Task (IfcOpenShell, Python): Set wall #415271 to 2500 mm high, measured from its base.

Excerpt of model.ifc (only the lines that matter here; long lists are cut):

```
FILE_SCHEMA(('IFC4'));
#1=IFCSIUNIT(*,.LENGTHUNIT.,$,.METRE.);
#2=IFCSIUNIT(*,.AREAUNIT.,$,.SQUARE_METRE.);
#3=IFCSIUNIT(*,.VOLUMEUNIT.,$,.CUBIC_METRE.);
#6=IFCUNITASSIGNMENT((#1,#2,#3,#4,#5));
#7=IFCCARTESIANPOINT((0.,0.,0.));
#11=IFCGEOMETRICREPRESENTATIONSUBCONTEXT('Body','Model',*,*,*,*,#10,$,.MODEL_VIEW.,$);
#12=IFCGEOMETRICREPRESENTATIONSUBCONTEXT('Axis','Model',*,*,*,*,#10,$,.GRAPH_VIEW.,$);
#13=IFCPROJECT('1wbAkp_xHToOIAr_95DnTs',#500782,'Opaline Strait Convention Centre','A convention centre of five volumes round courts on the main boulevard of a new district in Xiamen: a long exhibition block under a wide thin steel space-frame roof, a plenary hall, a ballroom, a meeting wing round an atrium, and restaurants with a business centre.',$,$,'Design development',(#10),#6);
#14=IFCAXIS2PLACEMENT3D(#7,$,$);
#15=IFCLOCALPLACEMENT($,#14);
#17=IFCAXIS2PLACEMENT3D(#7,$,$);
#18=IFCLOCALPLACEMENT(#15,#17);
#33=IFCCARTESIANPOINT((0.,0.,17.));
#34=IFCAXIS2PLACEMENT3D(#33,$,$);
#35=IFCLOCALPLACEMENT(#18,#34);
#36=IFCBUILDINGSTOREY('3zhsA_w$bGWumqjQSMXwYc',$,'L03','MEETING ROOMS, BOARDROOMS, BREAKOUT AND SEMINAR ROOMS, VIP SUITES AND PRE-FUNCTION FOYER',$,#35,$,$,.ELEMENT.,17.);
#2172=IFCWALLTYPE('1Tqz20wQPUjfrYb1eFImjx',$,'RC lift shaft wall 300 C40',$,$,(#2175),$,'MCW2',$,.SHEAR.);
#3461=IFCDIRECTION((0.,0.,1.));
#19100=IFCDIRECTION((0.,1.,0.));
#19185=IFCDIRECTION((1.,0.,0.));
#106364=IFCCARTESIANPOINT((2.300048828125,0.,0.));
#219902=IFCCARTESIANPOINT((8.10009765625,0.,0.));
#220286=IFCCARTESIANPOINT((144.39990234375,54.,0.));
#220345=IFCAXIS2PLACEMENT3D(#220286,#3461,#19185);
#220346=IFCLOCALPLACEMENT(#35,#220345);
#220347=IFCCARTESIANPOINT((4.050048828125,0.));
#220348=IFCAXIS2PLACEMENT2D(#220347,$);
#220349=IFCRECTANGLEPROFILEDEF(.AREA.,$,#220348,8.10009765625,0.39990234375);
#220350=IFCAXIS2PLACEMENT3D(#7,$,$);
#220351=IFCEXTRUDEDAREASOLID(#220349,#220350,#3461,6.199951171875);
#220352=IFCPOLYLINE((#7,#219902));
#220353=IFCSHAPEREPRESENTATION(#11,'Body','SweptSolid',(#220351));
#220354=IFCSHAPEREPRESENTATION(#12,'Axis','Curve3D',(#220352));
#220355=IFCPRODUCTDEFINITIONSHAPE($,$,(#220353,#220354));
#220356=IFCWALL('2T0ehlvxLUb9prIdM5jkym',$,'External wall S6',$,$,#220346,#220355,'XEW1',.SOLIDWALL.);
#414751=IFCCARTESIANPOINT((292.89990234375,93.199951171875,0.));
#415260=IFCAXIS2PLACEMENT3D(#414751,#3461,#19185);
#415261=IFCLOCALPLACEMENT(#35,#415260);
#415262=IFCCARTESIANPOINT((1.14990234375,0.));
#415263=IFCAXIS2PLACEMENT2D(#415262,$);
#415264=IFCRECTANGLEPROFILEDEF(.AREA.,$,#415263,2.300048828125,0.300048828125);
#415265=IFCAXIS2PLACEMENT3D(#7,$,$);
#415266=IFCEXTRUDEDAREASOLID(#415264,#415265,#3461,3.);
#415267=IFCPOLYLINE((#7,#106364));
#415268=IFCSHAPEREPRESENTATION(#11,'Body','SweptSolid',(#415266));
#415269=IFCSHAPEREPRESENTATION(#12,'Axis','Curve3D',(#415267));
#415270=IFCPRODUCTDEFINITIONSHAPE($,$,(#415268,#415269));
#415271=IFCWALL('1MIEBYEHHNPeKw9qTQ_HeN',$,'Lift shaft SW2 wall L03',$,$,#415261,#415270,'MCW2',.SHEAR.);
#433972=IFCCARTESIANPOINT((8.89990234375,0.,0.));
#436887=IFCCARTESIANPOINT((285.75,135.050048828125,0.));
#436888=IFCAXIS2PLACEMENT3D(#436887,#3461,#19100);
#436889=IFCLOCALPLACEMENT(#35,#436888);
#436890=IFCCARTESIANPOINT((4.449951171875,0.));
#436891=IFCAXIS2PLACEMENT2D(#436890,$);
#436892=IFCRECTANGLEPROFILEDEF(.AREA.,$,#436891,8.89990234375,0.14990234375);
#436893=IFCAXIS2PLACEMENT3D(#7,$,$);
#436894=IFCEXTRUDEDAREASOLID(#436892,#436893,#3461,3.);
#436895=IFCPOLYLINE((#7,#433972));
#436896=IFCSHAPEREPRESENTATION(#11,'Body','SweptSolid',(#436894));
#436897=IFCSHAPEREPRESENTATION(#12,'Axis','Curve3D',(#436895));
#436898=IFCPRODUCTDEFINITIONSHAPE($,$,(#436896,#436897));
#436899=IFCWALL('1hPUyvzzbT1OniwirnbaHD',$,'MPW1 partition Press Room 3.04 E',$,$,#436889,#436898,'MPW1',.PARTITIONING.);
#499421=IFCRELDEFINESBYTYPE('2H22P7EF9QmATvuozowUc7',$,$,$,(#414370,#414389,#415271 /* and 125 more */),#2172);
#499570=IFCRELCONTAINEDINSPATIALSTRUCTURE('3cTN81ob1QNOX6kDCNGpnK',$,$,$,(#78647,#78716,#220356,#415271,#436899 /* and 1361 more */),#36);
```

```python
import ifcopenshell
import ifcopenshell.geom
import ifcopenshell.util.representation
import ifcopenshell.util.shape
import ifcopenshell.util.unit

model = ifcopenshell.open("model.ifc")
unit_scale = ifcopenshell.util.unit.calculate_unit_scale(model)
settings = ifcopenshell.geom.settings()


def volume(element):
    """Net volume in cubic metres, openings subtracted."""
    shape = ifcopenshell.geom.create_shape(settings, element)
    return ifcopenshell.util.shape.get_volume(shape.geometry)


wall = model.by_guid("1MIEBYEHHNPeKw9qTQ_HeN")
before = volume(wall)

body = ifcopenshell.util.representation.get_representation(wall, "Model", "Body")
solid = body.Items[0]
old_height = solid.Depth
solid.Depth = 2.5 / unit_scale
after = volume(wall)

print(f"height {old_height:g} -> {solid.Depth:g}, volume {before:.3f} -> {after:.3f} m3")

model.write("model_updated.ifc")
```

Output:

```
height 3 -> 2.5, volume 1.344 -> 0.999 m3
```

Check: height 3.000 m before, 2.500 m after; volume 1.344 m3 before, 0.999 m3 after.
